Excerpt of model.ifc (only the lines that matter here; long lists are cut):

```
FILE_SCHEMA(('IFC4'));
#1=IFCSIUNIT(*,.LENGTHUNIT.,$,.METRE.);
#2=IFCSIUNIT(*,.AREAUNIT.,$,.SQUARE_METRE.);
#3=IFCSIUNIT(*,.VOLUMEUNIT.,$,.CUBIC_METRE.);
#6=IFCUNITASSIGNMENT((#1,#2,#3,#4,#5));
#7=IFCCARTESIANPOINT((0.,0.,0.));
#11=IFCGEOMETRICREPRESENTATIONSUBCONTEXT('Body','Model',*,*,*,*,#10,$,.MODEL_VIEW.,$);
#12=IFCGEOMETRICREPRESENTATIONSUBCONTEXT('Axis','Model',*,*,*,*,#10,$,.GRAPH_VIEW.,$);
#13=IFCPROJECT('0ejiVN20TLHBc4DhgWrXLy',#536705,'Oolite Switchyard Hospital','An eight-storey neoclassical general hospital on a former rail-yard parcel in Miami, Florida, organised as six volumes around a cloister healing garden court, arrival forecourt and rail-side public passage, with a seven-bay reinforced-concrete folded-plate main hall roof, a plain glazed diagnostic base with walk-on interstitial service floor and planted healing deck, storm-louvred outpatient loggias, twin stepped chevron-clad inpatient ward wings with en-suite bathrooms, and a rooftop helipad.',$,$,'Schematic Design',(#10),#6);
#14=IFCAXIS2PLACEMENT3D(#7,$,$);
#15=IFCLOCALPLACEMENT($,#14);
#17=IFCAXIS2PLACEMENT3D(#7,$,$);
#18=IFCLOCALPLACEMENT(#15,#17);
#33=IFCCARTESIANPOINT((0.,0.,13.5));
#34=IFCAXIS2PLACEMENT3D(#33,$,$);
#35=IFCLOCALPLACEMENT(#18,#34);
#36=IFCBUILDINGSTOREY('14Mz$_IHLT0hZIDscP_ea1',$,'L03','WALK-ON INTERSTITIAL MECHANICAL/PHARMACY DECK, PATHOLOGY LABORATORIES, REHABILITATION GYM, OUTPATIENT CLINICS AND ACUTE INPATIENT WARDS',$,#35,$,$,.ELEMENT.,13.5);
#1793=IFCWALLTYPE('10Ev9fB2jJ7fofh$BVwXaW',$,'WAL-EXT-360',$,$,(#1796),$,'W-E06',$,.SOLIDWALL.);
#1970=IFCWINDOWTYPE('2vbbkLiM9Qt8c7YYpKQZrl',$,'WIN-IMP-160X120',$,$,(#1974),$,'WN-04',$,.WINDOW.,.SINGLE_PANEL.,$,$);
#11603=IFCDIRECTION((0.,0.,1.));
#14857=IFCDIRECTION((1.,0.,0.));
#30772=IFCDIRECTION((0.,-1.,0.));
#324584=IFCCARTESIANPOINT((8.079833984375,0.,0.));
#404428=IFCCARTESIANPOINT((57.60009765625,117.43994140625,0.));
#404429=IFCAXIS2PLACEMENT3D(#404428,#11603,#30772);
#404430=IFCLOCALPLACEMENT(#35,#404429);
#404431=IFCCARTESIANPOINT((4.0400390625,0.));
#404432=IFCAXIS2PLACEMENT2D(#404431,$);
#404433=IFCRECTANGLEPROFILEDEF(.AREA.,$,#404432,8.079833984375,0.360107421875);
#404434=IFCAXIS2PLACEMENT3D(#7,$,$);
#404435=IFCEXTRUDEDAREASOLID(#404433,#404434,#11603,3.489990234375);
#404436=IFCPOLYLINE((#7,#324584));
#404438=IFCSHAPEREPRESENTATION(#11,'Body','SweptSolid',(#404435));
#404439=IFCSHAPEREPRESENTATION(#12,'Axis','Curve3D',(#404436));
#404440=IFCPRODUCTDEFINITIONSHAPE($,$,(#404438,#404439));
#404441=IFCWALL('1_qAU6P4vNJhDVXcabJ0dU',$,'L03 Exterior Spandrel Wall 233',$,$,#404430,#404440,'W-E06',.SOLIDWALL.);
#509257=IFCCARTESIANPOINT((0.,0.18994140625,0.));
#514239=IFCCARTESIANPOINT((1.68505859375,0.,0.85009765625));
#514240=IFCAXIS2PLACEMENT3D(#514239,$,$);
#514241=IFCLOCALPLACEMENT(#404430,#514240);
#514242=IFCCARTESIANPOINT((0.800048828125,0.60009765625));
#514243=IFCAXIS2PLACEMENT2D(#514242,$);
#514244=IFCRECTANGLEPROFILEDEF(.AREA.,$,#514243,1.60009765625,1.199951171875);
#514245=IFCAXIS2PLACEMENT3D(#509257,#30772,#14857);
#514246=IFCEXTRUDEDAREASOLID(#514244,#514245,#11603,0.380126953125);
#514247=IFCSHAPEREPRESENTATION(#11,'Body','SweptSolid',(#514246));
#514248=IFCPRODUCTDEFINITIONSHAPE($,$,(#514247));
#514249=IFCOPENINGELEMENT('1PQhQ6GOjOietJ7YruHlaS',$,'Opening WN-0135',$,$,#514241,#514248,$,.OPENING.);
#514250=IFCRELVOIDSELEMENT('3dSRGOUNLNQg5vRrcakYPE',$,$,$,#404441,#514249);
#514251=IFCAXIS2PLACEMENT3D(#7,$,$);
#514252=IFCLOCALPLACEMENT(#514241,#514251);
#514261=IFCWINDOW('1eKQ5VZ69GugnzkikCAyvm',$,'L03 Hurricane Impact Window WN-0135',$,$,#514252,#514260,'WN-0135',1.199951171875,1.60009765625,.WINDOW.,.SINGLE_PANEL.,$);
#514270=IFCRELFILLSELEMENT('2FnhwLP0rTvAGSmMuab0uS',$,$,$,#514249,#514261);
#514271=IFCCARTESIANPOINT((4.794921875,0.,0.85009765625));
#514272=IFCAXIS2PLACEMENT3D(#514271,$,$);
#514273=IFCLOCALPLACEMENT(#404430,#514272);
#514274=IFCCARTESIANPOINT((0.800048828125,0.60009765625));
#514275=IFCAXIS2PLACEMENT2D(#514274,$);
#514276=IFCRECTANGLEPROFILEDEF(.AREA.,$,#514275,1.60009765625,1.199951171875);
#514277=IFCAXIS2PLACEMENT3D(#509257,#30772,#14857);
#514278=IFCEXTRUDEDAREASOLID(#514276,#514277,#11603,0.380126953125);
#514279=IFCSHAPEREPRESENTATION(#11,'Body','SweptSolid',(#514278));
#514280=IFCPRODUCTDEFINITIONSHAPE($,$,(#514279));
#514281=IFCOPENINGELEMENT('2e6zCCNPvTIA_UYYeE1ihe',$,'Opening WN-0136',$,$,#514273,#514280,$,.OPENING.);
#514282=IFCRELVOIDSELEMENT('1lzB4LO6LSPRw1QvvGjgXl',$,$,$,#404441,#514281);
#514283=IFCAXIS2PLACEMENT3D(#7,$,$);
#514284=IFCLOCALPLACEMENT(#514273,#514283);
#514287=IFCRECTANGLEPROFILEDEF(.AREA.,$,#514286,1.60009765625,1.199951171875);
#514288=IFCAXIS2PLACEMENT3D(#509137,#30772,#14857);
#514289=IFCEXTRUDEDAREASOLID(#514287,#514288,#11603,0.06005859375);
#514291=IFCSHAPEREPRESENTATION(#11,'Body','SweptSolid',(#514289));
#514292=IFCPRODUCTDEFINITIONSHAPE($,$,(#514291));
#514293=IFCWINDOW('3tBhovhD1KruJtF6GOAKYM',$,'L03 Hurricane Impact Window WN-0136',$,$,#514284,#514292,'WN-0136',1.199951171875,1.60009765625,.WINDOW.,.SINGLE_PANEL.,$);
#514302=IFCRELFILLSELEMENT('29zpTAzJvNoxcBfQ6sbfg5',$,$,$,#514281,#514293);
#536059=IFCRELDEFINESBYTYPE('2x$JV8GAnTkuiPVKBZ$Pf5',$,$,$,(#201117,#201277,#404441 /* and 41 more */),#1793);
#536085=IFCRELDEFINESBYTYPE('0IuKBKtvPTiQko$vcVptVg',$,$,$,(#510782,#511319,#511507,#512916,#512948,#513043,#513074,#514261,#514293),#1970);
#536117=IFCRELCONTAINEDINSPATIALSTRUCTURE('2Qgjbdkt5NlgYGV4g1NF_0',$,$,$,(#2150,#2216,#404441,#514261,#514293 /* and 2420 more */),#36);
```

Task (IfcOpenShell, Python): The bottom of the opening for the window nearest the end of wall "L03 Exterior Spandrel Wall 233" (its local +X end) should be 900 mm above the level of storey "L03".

```python
import numpy as np
import ifcopenshell
import ifcopenshell.api.geometry
import ifcopenshell.geom
import ifcopenshell.util.element
import ifcopenshell.util.placement
import ifcopenshell.util.shape
import ifcopenshell.util.unit

model = ifcopenshell.open("model.ifc")
unit_scale = ifcopenshell.util.unit.calculate_unit_scale(model)

window = model.by_guid("3tBhovhD1KruJtF6GOAKYM")
opening = window.FillsVoids[0].RelatingOpeningElement
storey = ifcopenshell.util.element.get_container(window, ifc_class="IfcBuildingStorey")
level = ifcopenshell.util.placement.get_local_placement(storey.ObjectPlacement)[2, 3]

# The opening's origin need not be at the sill, so measure its lowest point.
shape = ifcopenshell.geom.create_shape(ifcopenshell.geom.settings(), opening)
bottom = ifcopenshell.util.shape.get_shape_bottom_elevation(shape, shape.geometry) / unit_scale
dz = level + 0.9 / unit_scale - bottom

shift = np.array([0.0, 0.0, dz])
# The window is placed relative to its opening, so it follows when the opening moves.
matrix = ifcopenshell.util.placement.get_local_placement(opening.ObjectPlacement)
matrix[:3, 3] += shift
ifcopenshell.api.geometry.edit_object_placement(
    model, product=opening, matrix=matrix, is_si=False, should_transform_children=True
)

print(f"moved by {dz * unit_scale:+.3f} m")

model.write("model_v2.ifc")
```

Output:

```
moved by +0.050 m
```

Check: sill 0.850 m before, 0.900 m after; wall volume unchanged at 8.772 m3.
